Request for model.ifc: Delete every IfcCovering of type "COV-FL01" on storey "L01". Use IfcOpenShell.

First a look at what the model holds.

```python
import ifcopenshell
import ifcopenshell.util.element

model = ifcopenshell.open("model.ifc")
print(model.schema)
storey = next(s for s in model.by_type("IfcBuildingStorey") if s.Name == "L01")
coverings = [e for e in ifcopenshell.util.element.get_decomposition(storey) if e.is_a("IfcCovering")]
seen = {}
for e in coverings:
    element_type = ifcopenshell.util.element.get_type(e)
    name = element_type.Name if element_type not in (None, e) else None
    seen[name] = seen.get(name, 0) + 1
for name, count in sorted(seen.items(), key=str):
    print(count, "x", name)
```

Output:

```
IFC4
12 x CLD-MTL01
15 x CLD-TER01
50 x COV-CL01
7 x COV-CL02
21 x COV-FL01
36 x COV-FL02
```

```python
import ifcopenshell
import ifcopenshell.api.root
import ifcopenshell.util.element

model = ifcopenshell.open("model.ifc")

storey = next(s for s in model.by_type("IfcBuildingStorey") if s.Name == "L01")
coverings = [e for e in ifcopenshell.util.element.get_decomposition(storey) if e.is_a("IfcCovering")]
targets = [e for e in coverings if (t := ifcopenshell.util.element.get_type(e)) not in (None, e) and t.Name == "COV-FL01"]

for e in targets:
    ifcopenshell.api.root.remove_product(model, product=e)
print(len(targets), "removed")

model.write("model_rev.ifc")
```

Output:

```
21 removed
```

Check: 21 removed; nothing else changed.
